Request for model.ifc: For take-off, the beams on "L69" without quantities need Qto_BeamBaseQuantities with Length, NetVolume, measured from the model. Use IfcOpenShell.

First a look at what the model holds.

```python
import ifcopenshell
import ifcopenshell.util.element
import ifcopenshell.util.unit

model = ifcopenshell.open("model.ifc")
print(model.schema)
for unit_type in ("LENGTHUNIT", "AREAUNIT", "VOLUMEUNIT"):
    print(unit_type, ifcopenshell.util.unit.calculate_unit_scale(model, unit_type))
storey = next(s for s in model.by_type("IfcBuildingStorey") if s.Name == "L69")
beams = [e for e in ifcopenshell.util.element.get_decomposition(storey) if e.is_a("IfcBeam")]
for e in sorted(beams, key=lambda e: e.id()):
    print(e.id(), e.is_a(), e.Name, list(ifcopenshell.util.element.get_psets(e, qtos_only=True)), sep=" | ")
```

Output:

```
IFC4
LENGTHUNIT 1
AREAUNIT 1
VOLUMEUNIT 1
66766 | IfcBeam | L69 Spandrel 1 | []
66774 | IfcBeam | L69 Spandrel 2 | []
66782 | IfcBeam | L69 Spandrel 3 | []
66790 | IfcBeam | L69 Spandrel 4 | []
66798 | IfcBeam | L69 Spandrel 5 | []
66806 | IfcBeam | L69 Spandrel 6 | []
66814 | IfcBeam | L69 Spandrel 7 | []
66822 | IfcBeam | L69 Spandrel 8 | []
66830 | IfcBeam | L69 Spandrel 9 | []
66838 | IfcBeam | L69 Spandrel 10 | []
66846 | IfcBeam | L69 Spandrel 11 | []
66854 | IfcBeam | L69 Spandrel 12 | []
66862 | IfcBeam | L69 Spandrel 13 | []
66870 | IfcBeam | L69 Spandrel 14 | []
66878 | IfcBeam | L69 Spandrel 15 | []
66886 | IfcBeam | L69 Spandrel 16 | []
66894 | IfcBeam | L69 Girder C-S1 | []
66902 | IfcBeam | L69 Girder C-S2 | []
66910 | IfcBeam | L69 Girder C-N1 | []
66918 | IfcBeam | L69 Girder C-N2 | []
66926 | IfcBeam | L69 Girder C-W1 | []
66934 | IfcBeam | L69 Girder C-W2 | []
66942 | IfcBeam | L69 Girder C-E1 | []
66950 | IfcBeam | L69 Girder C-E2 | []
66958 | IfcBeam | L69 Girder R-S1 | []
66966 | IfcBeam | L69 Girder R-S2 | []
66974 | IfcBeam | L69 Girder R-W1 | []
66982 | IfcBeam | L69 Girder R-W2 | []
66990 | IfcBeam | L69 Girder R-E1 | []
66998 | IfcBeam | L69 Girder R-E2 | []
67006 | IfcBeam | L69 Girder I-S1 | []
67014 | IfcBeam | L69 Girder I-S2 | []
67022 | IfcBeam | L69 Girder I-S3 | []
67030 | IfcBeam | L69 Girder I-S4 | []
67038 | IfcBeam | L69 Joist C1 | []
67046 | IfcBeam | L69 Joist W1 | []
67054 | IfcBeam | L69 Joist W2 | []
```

```python
import ifcopenshell
import ifcopenshell.api.pset
import ifcopenshell.geom
import ifcopenshell.util.element
import ifcopenshell.util.shape
import ifcopenshell.util.unit

model = ifcopenshell.open("model.ifc")
unit_scale = ifcopenshell.util.unit.calculate_unit_scale(model)
volume_scale = ifcopenshell.util.unit.calculate_unit_scale(model, "VOLUMEUNIT")
settings = ifcopenshell.geom.settings()

storey = next(s for s in model.by_type("IfcBuildingStorey") if s.Name == "L69")
beams = [e for e in ifcopenshell.util.element.get_decomposition(storey) if e.is_a("IfcBeam")]

for e in sorted(beams, key=lambda e: e.id()):
    if ifcopenshell.util.element.get_psets(e, qtos_only=True, should_inherit=False):
        continue
    # Geometry comes back in metres, in the element's own axes.
    shape = ifcopenshell.geom.create_shape(settings, e)
    values = {
        "Length": ifcopenshell.util.shape.get_max_xyz(shape.geometry) / unit_scale,
        "NetVolume": ifcopenshell.util.shape.get_volume(shape.geometry) / volume_scale,
    }
    qto = ifcopenshell.api.pset.add_qto(model, product=e, name="Qto_BeamBaseQuantities")
    ifcopenshell.api.pset.edit_qto(model, qto=qto, properties=values)
    print(e.id(), {k: round(v, 3) for k, v in values.items()})

model.write("model_v2.ifc")
```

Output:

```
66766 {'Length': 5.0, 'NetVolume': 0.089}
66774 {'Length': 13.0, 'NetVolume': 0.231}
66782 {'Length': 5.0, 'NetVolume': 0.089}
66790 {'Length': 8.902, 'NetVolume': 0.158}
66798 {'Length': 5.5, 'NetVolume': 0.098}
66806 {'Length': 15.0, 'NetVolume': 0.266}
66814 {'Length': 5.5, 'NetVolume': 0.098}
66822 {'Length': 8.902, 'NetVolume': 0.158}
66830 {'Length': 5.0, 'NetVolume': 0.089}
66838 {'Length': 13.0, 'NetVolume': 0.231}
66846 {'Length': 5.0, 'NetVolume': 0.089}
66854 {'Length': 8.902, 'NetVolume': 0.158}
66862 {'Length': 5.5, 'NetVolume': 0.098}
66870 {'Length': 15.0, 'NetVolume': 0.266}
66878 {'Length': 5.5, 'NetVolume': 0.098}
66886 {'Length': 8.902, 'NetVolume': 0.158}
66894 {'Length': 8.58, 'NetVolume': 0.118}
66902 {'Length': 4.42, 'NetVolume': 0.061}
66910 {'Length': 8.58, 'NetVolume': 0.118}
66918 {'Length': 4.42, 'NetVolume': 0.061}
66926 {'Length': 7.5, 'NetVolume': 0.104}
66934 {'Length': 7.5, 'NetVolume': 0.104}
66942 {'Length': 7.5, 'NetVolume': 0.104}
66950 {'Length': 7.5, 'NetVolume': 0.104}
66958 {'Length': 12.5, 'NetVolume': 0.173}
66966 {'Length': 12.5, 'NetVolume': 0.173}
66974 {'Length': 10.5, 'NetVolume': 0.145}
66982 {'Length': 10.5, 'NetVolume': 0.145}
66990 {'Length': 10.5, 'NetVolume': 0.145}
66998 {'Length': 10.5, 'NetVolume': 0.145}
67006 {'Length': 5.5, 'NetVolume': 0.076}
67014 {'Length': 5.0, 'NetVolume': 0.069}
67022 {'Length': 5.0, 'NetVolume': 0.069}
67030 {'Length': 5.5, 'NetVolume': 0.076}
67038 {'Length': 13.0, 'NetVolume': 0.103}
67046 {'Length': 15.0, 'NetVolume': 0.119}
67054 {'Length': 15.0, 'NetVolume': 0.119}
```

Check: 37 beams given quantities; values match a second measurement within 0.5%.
